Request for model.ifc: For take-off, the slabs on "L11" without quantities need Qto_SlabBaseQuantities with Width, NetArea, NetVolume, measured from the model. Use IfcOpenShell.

First a look at what the model holds.

```python
import ifcopenshell
import ifcopenshell.util.element
import ifcopenshell.util.unit

model = ifcopenshell.open("model.ifc")
print(model.schema)
for unit_type in ("LENGTHUNIT", "AREAUNIT", "VOLUMEUNIT"):
    print(unit_type, ifcopenshell.util.unit.calculate_unit_scale(model, unit_type))
storey = next(s for s in model.by_type("IfcBuildingStorey") if s.Name == "L11")
slabs = [e for e in ifcopenshell.util.element.get_decomposition(storey) if e.is_a("IfcSlab")]
for e in sorted(slabs, key=lambda e: e.id()):
    print(e.id(), e.is_a(), e.Name, list(ifcopenshell.util.element.get_psets(e, qtos_only=True)), sep=" | ")
```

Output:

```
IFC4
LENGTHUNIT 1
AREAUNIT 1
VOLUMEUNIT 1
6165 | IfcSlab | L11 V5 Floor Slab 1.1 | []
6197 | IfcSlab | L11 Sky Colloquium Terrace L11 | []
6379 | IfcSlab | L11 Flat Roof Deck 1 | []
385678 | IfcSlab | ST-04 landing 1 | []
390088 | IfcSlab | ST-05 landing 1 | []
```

```python
import ifcopenshell
import ifcopenshell.api.pset
import ifcopenshell.geom
import ifcopenshell.util.element
import ifcopenshell.util.shape
import ifcopenshell.util.unit

model = ifcopenshell.open("model.ifc")
unit_scale = ifcopenshell.util.unit.calculate_unit_scale(model)
area_scale = ifcopenshell.util.unit.calculate_unit_scale(model, "AREAUNIT")
volume_scale = ifcopenshell.util.unit.calculate_unit_scale(model, "VOLUMEUNIT")
settings = ifcopenshell.geom.settings()

storey = next(s for s in model.by_type("IfcBuildingStorey") if s.Name == "L11")
slabs = [e for e in ifcopenshell.util.element.get_decomposition(storey) if e.is_a("IfcSlab")]

for e in sorted(slabs, key=lambda e: e.id()):
    if ifcopenshell.util.element.get_psets(e, qtos_only=True, should_inherit=False):
        continue
    # Geometry comes back in metres, in the element's own axes.
    shape = ifcopenshell.geom.create_shape(settings, e)
    values = {
        "Width": ifcopenshell.util.shape.get_z(shape.geometry) / unit_scale,
        "NetArea": ifcopenshell.util.shape.get_footprint_area(shape.geometry) / area_scale,
        "NetVolume": ifcopenshell.util.shape.get_volume(shape.geometry) / volume_scale,
    }
    qto = ifcopenshell.api.pset.add_qto(model, product=e, name="Qto_SlabBaseQuantities")
    ifcopenshell.api.pset.edit_qto(model, qto=qto, properties=values)
    print(e.id(), {k: round(v, 3) for k, v in values.items()})

model.write("model_rev.ifc")
```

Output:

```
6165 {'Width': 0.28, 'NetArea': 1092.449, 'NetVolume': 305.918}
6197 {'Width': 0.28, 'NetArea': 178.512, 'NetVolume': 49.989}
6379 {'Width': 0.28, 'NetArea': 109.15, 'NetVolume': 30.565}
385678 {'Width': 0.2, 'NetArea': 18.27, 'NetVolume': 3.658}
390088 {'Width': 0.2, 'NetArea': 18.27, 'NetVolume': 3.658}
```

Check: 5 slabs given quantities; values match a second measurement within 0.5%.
